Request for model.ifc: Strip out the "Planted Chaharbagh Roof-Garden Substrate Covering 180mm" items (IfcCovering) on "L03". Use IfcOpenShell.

First a look at what the model holds.

```python
import ifcopenshell
import ifcopenshell.util.element

model = ifcopenshell.open("model.ifc")
print(model.schema)
storey = next(s for s in model.by_type("IfcBuildingStorey") if s.Name == "L03")
coverings = [e for e in ifcopenshell.util.element.get_decomposition(storey) if e.is_a("IfcCovering")]
seen = {}
for e in coverings:
    element_type = ifcopenshell.util.element.get_type(e)
    name = element_type.Name if element_type not in (None, e) else None
    seen[name] = seen.get(name, 0) + 1
for name, count in sorted(seen.items(), key=str):
    print(count, "x", name)
```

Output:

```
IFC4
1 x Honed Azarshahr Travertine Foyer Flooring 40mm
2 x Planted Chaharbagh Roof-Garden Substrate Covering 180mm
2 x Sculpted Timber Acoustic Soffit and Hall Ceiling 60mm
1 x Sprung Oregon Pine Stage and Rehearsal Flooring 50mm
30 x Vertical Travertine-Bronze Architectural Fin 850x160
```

```python
import ifcopenshell
import ifcopenshell.api.root
import ifcopenshell.util.element

model = ifcopenshell.open("model.ifc")

storey = next(s for s in model.by_type("IfcBuildingStorey") if s.Name == "L03")
coverings = [e for e in ifcopenshell.util.element.get_decomposition(storey) if e.is_a("IfcCovering")]
targets = [e for e in coverings if (t := ifcopenshell.util.element.get_type(e)) not in (None, e) and t.Name == "Planted Chaharbagh Roof-Garden Substrate Covering 180mm"]

for e in targets:
    ifcopenshell.api.root.remove_product(model, product=e)
print(len(targets), "removed")

model.write("model_v2.ifc")
```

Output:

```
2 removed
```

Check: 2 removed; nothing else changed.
